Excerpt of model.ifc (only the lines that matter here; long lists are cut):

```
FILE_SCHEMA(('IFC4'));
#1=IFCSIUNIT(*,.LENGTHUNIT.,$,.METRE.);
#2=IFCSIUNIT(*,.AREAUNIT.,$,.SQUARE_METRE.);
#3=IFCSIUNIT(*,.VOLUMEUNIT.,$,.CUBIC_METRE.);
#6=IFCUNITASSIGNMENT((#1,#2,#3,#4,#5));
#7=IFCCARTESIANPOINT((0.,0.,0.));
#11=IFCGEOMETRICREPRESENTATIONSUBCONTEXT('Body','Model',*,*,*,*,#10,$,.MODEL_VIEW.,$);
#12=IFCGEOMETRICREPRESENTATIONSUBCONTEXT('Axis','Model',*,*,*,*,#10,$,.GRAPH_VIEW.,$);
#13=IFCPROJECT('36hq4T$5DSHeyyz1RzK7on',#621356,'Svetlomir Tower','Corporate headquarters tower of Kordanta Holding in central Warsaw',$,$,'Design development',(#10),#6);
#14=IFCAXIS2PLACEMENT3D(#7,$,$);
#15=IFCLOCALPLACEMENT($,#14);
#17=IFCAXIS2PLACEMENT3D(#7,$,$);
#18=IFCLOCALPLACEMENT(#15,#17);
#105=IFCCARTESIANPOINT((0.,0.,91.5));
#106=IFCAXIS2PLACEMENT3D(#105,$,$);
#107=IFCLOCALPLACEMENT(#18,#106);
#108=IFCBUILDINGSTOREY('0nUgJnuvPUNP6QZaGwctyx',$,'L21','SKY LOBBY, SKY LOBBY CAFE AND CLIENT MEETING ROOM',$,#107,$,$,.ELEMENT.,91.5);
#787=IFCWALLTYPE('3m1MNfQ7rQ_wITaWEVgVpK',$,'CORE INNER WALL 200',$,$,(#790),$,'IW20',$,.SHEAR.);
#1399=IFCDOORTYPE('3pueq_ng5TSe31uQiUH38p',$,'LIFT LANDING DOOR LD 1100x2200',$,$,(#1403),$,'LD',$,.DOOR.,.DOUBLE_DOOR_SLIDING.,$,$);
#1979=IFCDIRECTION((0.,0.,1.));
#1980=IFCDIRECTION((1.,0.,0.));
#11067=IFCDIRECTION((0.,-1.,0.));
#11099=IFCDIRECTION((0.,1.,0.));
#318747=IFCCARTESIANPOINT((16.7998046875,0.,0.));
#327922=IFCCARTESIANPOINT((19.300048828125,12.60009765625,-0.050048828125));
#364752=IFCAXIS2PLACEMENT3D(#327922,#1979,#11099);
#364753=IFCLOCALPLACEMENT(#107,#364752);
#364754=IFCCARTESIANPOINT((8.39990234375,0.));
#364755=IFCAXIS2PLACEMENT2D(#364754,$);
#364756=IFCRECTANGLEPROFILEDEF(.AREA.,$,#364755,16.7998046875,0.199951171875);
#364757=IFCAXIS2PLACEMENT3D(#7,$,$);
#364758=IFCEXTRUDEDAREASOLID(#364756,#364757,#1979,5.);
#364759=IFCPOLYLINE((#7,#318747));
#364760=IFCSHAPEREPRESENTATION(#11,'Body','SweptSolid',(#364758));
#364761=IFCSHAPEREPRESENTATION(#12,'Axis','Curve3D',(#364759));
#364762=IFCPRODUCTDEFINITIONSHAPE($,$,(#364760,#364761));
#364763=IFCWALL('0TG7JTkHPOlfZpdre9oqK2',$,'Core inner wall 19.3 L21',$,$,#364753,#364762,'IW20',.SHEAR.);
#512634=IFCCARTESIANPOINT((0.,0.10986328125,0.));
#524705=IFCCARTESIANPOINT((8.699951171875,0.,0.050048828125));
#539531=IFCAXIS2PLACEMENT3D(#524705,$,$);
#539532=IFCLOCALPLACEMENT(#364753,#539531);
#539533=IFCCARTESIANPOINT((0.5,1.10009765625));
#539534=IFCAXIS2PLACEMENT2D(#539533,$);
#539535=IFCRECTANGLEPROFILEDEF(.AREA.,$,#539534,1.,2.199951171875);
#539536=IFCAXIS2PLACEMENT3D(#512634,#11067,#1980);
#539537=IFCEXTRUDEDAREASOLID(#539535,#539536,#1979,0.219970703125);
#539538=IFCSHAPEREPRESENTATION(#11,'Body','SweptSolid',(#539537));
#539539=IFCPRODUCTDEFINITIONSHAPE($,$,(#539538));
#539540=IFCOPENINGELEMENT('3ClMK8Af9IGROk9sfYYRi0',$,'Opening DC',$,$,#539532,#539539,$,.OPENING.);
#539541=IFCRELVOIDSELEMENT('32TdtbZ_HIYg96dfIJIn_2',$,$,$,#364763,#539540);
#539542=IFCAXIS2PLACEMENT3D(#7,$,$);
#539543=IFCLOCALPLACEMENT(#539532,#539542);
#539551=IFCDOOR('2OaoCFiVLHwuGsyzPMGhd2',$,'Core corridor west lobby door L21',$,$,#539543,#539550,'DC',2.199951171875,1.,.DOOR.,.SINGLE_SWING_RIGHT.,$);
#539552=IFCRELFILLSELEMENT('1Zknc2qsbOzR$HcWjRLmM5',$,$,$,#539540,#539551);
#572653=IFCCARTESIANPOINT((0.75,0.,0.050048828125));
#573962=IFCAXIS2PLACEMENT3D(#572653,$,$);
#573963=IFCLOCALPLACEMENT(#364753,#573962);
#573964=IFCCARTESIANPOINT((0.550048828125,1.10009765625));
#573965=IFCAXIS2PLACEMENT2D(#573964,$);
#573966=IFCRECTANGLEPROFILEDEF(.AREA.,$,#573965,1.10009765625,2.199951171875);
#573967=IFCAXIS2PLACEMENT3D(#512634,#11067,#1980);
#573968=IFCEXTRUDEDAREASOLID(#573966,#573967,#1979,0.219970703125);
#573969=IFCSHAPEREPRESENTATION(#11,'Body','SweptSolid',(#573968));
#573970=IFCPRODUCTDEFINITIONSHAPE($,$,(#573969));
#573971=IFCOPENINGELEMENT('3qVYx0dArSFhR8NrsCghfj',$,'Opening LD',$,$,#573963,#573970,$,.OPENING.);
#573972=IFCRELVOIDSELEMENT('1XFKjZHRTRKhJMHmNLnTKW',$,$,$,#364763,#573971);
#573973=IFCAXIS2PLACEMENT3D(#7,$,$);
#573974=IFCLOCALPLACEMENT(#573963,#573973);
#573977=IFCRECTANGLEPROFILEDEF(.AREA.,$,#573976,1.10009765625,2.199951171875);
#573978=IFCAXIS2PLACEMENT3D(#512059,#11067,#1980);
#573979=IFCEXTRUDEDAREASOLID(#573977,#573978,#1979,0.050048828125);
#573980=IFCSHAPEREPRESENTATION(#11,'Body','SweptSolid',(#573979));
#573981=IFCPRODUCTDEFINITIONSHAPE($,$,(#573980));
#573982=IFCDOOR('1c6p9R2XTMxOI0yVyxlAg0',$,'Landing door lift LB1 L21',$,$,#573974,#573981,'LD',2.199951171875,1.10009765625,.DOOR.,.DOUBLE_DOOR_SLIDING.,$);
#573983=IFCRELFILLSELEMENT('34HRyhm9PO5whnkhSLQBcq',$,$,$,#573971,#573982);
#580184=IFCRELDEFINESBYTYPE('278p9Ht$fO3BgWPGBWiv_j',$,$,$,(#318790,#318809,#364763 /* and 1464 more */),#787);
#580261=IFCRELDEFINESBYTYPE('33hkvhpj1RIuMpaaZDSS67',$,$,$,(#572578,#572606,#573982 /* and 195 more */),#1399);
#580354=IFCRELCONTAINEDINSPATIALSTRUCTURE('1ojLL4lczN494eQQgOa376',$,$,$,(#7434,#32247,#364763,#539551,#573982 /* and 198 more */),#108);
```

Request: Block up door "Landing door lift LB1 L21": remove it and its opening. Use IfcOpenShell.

```python
import ifcopenshell
import ifcopenshell.api.feature
import ifcopenshell.api.root
import ifcopenshell.geom
import ifcopenshell.util.shape

model = ifcopenshell.open("model.ifc")
settings = ifcopenshell.geom.settings()


def volume(element):
    """Net volume in cubic metres, openings subtracted."""
    shape = ifcopenshell.geom.create_shape(settings, element)
    return ifcopenshell.util.shape.get_volume(shape.geometry)


door = model.by_guid("1c6p9R2XTMxOI0yVyxlAg0")
opening = door.FillsVoids[0].RelatingOpeningElement
wall = opening.VoidsElements[0].RelatingBuildingElement
before = volume(wall)

ifcopenshell.api.root.remove_product(model, product=door)
ifcopenshell.api.feature.remove_feature(model, feature=opening)

after = volume(wall)

print(f"wall volume {before:.3f} -> {after:.3f} m3")

model.write("model_v2.ifc")
```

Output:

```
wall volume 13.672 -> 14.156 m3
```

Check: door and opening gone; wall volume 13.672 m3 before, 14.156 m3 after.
